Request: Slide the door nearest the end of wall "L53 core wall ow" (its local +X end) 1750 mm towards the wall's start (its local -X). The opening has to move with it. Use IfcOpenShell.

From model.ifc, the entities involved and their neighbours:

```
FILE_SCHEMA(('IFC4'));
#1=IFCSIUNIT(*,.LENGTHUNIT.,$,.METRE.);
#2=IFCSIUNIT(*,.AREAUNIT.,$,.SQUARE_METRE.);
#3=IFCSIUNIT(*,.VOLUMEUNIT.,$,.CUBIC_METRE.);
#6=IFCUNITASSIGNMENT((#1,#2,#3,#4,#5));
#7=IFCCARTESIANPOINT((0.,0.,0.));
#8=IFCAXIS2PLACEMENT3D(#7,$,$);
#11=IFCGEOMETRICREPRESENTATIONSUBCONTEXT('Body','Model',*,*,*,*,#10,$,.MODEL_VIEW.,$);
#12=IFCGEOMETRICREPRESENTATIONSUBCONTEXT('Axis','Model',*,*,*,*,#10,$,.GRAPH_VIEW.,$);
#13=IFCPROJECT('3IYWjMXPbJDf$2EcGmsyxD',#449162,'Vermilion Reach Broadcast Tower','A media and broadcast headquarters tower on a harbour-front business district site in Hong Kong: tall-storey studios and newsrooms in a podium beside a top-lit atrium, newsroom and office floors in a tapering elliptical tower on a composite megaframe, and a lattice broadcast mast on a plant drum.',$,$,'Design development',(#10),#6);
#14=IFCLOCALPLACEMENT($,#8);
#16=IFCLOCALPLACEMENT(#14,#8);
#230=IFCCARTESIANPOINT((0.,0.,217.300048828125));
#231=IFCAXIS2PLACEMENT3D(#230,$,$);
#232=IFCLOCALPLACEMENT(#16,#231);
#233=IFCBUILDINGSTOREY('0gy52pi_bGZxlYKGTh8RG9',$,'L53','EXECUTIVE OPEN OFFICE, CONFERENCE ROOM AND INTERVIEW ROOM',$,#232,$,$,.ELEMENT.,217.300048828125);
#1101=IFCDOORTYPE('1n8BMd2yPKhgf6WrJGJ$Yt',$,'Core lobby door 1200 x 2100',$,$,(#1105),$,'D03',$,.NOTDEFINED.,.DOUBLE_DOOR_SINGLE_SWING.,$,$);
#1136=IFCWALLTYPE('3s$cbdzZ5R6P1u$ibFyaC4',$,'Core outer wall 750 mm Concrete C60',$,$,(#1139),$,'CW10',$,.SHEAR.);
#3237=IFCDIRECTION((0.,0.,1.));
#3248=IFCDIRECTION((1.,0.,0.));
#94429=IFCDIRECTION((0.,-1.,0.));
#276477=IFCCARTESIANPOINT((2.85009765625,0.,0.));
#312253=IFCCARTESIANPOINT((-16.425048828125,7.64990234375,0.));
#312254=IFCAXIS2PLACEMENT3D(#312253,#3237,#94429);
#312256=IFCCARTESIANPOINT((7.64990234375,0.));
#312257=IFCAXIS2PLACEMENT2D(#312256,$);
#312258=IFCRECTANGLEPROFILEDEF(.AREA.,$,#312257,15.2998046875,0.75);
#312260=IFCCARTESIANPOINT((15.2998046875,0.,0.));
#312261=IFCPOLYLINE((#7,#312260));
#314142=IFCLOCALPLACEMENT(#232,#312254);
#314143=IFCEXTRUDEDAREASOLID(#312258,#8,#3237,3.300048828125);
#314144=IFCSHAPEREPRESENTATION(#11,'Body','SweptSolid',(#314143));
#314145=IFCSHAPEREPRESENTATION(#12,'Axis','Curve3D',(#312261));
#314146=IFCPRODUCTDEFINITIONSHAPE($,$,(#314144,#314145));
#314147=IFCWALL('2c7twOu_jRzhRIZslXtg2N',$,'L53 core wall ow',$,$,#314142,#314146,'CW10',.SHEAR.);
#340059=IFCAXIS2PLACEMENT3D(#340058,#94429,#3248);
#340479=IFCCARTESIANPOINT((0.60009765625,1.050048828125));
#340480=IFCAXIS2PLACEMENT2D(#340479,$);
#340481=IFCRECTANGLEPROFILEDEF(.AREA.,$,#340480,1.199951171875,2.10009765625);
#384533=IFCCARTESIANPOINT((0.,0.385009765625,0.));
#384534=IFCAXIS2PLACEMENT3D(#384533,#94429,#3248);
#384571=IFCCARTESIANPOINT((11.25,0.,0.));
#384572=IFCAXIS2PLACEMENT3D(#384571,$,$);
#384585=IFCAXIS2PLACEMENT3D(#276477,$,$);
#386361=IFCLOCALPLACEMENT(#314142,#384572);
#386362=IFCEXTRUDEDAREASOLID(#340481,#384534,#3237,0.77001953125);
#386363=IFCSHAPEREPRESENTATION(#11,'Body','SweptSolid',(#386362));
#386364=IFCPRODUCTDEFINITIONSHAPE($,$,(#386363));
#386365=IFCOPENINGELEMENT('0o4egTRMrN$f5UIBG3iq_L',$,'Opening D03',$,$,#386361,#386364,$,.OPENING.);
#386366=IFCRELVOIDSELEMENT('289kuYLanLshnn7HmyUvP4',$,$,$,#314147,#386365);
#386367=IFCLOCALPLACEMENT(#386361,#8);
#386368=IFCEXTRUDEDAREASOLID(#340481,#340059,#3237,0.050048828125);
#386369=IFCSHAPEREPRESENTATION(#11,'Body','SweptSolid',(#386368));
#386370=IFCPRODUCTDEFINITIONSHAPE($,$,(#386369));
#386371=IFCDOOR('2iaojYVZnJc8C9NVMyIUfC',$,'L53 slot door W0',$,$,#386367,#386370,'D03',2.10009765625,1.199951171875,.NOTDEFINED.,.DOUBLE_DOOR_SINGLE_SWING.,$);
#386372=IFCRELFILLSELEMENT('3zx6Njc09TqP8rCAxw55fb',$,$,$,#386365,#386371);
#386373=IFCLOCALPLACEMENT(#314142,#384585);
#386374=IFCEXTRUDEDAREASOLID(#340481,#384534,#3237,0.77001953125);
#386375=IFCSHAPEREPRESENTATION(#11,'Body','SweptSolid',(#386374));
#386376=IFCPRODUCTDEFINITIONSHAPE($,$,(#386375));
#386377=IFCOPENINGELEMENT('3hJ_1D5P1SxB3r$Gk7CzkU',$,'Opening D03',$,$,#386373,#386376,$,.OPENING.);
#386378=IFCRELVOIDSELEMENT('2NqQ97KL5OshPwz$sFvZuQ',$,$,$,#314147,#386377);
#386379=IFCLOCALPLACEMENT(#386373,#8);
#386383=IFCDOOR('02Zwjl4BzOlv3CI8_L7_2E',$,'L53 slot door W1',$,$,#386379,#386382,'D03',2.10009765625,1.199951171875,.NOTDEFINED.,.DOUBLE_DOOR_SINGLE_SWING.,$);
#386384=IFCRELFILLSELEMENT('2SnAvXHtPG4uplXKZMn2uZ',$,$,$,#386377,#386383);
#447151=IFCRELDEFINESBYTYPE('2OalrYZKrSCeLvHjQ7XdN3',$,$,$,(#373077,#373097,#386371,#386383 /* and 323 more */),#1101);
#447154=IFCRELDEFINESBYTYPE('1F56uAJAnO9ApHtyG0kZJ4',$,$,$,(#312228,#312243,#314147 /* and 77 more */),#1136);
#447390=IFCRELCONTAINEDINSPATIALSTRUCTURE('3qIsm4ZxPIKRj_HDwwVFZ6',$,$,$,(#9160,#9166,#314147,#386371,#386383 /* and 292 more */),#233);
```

```python
import ifcopenshell
import ifcopenshell.api.geometry
import ifcopenshell.util.placement
import ifcopenshell.util.unit

model = ifcopenshell.open("model.ifc")
unit_scale = ifcopenshell.util.unit.calculate_unit_scale(model)

door = model.by_id(386371)
opening = door.FillsVoids[0].RelatingOpeningElement
wall = opening.VoidsElements[0].RelatingBuildingElement

wall_matrix = ifcopenshell.util.placement.get_local_placement(wall.ObjectPlacement)
shift = wall_matrix[:3, 0] * -1.75 / unit_scale
before = ifcopenshell.util.placement.get_local_placement(door.ObjectPlacement)[:3, 3].copy()

# The door is placed relative to its opening, so it follows when the opening moves.
matrix = ifcopenshell.util.placement.get_local_placement(opening.ObjectPlacement)
matrix[:3, 3] += shift
ifcopenshell.api.geometry.edit_object_placement(
    model, product=opening, matrix=matrix, is_si=False, should_transform_children=True
)

after = ifcopenshell.util.placement.get_local_placement(door.ObjectPlacement)[:3, 3]
print("door moved by", (after - before).round(3) + 0.0)

model.write("model-out.ifc")
```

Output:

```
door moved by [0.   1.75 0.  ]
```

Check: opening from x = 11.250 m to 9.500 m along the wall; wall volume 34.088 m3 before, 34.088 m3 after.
